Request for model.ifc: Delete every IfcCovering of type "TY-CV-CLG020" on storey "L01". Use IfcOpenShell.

First a look at what the model holds.

```python
import ifcopenshell
import ifcopenshell.util.element

model = ifcopenshell.open("model.ifc")
print(model.schema)
storey = next(s for s in model.by_type("IfcBuildingStorey") if s.Name == "L01")
coverings = [e for e in ifcopenshell.util.element.get_decomposition(storey) if e.is_a("IfcCovering")]
seen = {}
for e in coverings:
    element_type = ifcopenshell.util.element.get_type(e)
    name = element_type.Name if element_type not in (None, e) else None
    seen[name] = seen.get(name, 0) + 1
for name, count in sorted(seen.items(), key=str):
    print(count, "x", name)
```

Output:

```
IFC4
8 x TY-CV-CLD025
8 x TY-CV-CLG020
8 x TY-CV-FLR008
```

```python
import ifcopenshell
import ifcopenshell.api.root
import ifcopenshell.util.element

model = ifcopenshell.open("model.ifc")

storey = next(s for s in model.by_type("IfcBuildingStorey") if s.Name == "L01")
coverings = [e for e in ifcopenshell.util.element.get_decomposition(storey) if e.is_a("IfcCovering")]
targets = [e for e in coverings if (t := ifcopenshell.util.element.get_type(e)) not in (None, e) and t.Name == "TY-CV-CLG020"]

for e in targets:
    ifcopenshell.api.root.remove_product(model, product=e)
print(len(targets), "removed")

model.write("model_rev.ifc")
```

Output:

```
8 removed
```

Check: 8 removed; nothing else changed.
